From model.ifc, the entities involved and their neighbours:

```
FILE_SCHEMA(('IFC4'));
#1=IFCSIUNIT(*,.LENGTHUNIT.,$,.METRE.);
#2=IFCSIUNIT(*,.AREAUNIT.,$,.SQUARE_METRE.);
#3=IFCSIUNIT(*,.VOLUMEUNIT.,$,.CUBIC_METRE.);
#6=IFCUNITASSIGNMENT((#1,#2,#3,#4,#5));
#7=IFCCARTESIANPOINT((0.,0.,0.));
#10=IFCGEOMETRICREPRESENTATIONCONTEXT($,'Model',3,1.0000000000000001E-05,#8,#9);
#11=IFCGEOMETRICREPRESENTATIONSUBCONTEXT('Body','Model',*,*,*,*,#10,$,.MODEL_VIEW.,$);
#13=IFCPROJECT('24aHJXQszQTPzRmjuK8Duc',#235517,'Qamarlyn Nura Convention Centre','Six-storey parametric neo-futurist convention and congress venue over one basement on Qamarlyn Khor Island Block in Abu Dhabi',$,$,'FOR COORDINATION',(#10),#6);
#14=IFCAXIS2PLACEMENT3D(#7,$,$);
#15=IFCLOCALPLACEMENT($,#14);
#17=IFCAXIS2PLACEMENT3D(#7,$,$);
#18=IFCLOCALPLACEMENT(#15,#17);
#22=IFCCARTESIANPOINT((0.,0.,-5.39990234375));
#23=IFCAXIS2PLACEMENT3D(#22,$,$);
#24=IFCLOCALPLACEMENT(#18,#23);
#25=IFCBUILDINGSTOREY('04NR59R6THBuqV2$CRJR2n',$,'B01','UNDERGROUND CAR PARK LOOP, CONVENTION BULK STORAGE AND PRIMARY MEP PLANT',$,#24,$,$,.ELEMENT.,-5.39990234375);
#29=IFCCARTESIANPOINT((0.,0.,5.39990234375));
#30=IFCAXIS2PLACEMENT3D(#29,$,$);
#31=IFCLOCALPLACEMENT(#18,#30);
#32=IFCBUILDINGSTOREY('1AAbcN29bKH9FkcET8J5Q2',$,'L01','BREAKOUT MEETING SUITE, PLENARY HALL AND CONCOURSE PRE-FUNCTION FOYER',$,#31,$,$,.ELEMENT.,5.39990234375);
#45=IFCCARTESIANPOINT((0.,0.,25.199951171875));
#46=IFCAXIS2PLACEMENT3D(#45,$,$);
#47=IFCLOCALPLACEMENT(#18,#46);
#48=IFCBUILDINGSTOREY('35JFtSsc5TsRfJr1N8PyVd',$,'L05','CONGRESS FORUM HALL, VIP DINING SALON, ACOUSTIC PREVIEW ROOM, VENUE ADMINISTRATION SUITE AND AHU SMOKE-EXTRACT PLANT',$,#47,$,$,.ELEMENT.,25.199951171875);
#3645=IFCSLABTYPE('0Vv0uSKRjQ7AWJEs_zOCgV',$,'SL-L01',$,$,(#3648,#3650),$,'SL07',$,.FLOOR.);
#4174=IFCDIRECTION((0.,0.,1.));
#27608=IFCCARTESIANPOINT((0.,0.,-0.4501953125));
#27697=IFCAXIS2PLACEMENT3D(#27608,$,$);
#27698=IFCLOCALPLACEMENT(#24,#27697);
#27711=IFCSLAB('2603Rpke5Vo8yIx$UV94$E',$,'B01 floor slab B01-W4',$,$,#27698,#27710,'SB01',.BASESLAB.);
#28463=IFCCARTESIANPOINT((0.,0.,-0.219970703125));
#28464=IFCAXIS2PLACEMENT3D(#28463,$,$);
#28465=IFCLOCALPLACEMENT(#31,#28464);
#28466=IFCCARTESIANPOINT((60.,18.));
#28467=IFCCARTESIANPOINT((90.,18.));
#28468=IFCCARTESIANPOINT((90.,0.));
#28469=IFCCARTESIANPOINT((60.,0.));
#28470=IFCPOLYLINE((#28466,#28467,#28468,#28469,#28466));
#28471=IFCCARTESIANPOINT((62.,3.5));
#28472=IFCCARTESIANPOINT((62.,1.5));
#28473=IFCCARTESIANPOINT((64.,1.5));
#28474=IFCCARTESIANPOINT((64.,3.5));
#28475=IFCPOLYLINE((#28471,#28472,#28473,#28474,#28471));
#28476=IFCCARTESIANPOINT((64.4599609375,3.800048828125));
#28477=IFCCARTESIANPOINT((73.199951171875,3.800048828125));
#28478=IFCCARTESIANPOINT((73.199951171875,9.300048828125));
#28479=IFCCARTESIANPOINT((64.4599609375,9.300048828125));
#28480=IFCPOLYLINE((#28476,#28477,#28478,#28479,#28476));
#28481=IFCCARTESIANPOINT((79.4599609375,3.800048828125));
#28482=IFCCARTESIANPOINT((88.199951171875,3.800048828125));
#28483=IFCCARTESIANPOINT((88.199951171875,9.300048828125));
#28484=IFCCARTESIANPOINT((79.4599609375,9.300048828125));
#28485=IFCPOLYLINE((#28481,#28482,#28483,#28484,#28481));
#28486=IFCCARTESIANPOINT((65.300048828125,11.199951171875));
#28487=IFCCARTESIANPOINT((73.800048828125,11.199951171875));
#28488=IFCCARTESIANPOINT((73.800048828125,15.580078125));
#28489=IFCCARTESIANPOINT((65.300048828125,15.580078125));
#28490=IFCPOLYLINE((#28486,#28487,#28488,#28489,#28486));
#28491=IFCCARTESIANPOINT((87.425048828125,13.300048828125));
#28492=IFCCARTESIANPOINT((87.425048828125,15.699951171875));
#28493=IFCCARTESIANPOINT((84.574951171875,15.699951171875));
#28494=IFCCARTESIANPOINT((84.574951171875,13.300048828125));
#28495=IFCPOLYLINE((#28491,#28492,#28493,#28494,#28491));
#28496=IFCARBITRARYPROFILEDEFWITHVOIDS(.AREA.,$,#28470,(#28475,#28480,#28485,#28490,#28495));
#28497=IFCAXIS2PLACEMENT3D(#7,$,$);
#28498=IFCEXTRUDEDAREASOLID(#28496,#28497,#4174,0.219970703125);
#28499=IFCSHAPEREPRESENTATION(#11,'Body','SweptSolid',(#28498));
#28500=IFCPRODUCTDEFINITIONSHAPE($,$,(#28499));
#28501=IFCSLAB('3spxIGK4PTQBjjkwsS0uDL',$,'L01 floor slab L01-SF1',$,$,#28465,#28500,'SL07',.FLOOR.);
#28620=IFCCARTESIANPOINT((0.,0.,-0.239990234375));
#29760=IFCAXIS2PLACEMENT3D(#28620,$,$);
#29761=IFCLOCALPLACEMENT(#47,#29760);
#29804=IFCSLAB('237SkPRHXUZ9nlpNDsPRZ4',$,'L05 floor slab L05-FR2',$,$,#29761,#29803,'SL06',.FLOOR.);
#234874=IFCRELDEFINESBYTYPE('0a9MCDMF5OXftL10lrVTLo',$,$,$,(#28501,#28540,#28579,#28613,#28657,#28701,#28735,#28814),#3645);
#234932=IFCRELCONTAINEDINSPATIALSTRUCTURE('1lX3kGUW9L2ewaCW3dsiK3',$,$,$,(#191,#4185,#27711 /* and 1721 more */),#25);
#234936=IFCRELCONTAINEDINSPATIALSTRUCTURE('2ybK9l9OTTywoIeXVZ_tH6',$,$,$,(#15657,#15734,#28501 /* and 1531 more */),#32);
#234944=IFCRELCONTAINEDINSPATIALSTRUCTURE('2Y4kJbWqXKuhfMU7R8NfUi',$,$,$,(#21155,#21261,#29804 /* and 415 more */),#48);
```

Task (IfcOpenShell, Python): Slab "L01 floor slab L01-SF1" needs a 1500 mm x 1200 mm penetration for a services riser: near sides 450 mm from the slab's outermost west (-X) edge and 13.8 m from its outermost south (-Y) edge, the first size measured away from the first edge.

```python
import numpy as np
import ifcopenshell
import ifcopenshell.api.feature
import ifcopenshell.api.geometry
import ifcopenshell.api.root
import ifcopenshell.geom
import ifcopenshell.util.placement
import ifcopenshell.util.representation
import ifcopenshell.util.shape
import ifcopenshell.util.unit

model = ifcopenshell.open("model.ifc")
unit_scale = ifcopenshell.util.unit.calculate_unit_scale(model)
settings = ifcopenshell.geom.settings()


def volume(element):
    """Net volume in cubic metres, openings subtracted."""
    shape = ifcopenshell.geom.create_shape(settings, element)
    return ifcopenshell.util.shape.get_volume(shape.geometry)


slab = model.by_guid("3spxIGK4PTQBjjkwsS0uDL")
before = volume(slab)

# Extent in the slab's own axes, in metres. The edges named are its -X and -Y sides.
slab_shape = ifcopenshell.geom.create_shape(settings, slab)
vertices = ifcopenshell.util.shape.get_vertices(slab_shape.geometry)
x_min, y_min, bottom = vertices.min(axis=0)
top = vertices[:, 2].max()

opening = ifcopenshell.api.root.create_entity(model, ifc_class="IfcOpeningElement", name="Services riser opening", predefined_type="OPENING")
context = ifcopenshell.util.representation.get_context(model, "Model", "Body", "MODEL_VIEW")
width, depth = 1.5, 1.2
outline = [(0.0, 0.0), (width, 0.0), (width, depth), (0.0, depth), (0.0, 0.0)]
# Overshoot both faces by 50 mm so the cut is clean.
shape = ifcopenshell.api.geometry.add_slab_representation(
    model, context=context, depth=top - bottom + 0.1, polyline=outline
)
ifcopenshell.api.geometry.assign_representation(model, product=opening, representation=shape)

matrix = ifcopenshell.util.placement.get_local_placement(slab.ObjectPlacement)
matrix[:, 3] = matrix @ np.append(np.array([x_min + 0.45, y_min + 13.8, bottom - 0.05]) / unit_scale, 1.0)
ifcopenshell.api.geometry.edit_object_placement(model, product=opening, matrix=matrix, is_si=False)
ifcopenshell.api.feature.add_feature(model, feature=opening, element=slab)

after = volume(slab)

print(f"slab volume {before:.3f} -> {after:.3f} m3")

model.write("model-out.ifc")
```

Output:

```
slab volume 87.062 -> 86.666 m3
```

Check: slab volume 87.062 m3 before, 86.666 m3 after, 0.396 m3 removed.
